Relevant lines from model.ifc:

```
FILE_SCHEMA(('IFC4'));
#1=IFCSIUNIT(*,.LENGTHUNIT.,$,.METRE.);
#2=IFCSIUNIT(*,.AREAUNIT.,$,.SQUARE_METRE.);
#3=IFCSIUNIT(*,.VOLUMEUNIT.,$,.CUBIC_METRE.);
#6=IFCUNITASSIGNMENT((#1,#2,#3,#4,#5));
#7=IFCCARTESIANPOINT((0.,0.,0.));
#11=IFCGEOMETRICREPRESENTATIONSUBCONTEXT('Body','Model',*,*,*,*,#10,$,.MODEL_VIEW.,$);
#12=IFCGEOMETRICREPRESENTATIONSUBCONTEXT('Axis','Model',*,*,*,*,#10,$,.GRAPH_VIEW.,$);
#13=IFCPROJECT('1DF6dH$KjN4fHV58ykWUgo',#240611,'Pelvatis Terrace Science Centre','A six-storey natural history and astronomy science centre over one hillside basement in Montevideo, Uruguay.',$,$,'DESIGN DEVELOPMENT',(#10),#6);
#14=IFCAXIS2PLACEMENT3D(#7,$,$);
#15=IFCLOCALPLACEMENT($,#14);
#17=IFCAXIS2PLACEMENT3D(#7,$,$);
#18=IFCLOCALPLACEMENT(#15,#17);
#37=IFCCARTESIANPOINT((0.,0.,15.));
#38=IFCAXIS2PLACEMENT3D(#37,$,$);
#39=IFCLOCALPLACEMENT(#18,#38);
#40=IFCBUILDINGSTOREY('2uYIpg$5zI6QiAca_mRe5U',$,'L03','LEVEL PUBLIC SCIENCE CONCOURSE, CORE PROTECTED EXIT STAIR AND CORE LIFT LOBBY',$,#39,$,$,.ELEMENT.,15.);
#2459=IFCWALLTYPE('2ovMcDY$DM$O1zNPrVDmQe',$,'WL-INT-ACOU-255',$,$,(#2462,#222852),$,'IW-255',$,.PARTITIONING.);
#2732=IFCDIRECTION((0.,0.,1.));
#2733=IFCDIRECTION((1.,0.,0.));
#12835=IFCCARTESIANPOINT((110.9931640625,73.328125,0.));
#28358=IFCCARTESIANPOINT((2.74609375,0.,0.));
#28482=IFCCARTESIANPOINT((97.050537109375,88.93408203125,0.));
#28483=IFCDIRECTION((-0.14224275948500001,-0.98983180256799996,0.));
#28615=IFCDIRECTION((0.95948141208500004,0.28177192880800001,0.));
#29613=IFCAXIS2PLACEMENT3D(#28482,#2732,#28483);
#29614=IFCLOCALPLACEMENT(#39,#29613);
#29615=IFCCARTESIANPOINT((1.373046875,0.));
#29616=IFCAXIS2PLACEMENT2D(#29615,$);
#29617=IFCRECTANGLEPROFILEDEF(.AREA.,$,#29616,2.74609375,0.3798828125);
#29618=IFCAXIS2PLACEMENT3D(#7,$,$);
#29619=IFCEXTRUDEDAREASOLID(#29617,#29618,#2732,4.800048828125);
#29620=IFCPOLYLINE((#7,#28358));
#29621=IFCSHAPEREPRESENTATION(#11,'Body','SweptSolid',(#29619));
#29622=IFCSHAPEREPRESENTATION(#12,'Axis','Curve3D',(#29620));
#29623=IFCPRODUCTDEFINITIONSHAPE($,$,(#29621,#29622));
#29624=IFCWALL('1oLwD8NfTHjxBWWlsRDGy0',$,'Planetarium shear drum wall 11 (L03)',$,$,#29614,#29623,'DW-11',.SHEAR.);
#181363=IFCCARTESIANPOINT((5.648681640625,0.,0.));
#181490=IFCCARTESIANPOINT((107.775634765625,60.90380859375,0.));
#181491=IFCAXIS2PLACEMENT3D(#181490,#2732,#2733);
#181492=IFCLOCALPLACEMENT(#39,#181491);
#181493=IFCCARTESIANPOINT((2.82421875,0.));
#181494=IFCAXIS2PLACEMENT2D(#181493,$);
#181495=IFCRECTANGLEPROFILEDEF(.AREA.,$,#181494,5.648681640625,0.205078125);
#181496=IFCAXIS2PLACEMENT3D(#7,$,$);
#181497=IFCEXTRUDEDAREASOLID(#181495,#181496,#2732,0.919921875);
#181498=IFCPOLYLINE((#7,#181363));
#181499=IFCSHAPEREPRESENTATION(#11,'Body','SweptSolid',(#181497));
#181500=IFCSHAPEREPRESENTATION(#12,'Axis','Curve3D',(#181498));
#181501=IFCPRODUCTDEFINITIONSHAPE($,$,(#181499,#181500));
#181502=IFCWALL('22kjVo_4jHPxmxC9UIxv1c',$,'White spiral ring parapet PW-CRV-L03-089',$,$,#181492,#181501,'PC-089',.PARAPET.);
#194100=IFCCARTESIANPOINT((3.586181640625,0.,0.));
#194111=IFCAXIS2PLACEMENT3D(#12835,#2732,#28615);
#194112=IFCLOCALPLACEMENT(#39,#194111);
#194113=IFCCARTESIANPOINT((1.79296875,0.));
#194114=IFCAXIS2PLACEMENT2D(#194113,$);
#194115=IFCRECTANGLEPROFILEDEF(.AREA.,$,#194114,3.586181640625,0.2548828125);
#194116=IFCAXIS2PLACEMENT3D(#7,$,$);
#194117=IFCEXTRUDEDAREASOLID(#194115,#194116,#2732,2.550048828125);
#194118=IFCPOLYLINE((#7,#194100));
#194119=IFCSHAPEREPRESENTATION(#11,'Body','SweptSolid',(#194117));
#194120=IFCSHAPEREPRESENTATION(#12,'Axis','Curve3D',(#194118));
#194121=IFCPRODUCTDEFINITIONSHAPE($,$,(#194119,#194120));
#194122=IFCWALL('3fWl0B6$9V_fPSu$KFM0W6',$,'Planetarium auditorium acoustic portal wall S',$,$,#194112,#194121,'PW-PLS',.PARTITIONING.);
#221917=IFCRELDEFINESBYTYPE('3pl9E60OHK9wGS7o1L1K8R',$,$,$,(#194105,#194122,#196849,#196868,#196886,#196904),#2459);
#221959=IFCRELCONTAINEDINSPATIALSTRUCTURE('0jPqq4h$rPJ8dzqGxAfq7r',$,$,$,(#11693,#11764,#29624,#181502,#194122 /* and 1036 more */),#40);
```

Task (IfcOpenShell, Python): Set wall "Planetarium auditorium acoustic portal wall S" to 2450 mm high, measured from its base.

```python
import ifcopenshell
import ifcopenshell.geom
import ifcopenshell.util.representation
import ifcopenshell.util.shape

model = ifcopenshell.open("model.ifc")
settings = ifcopenshell.geom.settings()


def volume(element):
    """Net volume in cubic metres, openings subtracted."""
    shape = ifcopenshell.geom.create_shape(settings, element)
    return ifcopenshell.util.shape.get_volume(shape.geometry)


wall = model.by_guid("3fWl0B6$9V_fPSu$KFM0W6")
before = volume(wall)

body = ifcopenshell.util.representation.get_representation(wall, "Model", "Body")
solid = body.Items[0]
old_height = solid.Depth
solid.Depth = 2.45
after = volume(wall)

print(f"height {old_height:g} -> {solid.Depth:g}, volume {before:.3f} -> {after:.3f} m3")

model.write("model_rev.ifc")
```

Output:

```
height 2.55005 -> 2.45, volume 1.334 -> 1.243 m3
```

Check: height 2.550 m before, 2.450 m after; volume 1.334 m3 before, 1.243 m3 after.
